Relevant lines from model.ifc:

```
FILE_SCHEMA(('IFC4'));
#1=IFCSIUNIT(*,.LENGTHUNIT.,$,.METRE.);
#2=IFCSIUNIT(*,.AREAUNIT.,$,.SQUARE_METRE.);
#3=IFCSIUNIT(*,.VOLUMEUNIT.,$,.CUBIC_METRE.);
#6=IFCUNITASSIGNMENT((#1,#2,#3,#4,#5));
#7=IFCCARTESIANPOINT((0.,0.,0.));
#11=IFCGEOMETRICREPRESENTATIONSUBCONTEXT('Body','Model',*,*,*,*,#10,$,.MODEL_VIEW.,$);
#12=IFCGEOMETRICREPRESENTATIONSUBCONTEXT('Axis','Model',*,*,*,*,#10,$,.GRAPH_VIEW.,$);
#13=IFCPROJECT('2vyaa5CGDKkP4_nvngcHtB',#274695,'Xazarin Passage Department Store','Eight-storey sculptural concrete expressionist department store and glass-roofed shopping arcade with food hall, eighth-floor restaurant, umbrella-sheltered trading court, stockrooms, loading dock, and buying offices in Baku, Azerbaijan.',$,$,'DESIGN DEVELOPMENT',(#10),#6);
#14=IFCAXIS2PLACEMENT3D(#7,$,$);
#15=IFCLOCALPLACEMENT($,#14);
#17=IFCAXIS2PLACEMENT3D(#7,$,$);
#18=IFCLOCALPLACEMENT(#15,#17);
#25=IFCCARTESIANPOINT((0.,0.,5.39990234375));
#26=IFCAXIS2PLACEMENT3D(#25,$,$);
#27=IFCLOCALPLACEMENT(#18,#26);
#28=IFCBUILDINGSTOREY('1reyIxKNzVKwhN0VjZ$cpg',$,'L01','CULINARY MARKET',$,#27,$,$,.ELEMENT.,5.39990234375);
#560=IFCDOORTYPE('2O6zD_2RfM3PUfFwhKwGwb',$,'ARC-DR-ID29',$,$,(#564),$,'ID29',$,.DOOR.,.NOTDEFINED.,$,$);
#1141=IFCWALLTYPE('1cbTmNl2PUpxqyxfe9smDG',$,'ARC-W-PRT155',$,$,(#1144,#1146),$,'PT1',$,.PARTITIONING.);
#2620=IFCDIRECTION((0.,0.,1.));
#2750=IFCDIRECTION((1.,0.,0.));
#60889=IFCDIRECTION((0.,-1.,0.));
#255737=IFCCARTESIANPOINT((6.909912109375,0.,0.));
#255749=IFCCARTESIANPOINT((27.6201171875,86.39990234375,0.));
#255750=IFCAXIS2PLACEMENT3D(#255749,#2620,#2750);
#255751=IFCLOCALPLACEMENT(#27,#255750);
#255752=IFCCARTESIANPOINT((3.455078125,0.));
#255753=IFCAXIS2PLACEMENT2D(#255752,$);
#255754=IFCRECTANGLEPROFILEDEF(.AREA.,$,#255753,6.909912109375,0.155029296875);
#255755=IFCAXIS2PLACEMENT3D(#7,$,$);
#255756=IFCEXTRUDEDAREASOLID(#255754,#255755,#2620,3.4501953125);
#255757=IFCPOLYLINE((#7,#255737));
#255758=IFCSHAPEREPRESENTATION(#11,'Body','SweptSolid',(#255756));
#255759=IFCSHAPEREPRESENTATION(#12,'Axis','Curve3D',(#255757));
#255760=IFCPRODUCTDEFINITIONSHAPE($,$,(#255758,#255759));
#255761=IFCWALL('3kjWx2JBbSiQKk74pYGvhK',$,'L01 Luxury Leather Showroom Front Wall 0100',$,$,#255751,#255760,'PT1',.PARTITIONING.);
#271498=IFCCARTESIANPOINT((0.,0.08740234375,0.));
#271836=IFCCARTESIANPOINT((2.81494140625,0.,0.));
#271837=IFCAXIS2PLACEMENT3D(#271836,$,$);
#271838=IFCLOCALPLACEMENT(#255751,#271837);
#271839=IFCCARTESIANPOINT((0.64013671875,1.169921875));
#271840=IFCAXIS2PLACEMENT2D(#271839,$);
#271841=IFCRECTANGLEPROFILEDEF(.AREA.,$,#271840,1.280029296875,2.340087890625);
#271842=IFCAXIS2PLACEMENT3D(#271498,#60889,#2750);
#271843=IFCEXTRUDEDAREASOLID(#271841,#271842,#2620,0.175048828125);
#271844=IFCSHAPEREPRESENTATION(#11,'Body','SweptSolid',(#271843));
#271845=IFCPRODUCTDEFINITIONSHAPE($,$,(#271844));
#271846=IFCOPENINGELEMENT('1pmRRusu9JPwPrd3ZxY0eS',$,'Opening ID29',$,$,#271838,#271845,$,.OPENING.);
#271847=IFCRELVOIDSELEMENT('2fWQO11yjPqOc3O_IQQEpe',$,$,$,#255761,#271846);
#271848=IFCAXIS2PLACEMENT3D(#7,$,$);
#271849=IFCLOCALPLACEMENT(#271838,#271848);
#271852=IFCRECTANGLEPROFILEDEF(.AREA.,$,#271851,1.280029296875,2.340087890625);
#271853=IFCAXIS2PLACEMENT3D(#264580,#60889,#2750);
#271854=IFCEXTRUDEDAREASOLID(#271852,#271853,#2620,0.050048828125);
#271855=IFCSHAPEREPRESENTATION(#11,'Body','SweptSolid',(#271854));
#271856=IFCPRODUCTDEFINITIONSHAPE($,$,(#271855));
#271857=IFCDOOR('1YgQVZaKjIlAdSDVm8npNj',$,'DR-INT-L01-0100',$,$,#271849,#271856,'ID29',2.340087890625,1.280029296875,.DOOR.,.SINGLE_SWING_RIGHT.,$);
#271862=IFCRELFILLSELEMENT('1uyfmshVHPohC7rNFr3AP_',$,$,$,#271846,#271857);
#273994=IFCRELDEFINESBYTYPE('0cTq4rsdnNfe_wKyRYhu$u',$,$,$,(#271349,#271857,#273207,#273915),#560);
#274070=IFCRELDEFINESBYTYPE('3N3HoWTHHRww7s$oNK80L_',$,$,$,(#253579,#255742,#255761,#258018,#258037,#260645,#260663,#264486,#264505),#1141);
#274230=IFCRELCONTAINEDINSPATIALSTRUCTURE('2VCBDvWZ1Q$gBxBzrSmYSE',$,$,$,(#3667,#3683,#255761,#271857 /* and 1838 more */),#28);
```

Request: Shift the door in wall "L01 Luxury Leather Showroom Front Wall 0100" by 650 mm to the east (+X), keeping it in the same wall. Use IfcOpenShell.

```python
import ifcopenshell
import ifcopenshell.api.geometry
import ifcopenshell.util.placement
import ifcopenshell.util.unit

model = ifcopenshell.open("model.ifc")
unit_scale = ifcopenshell.util.unit.calculate_unit_scale(model)

door = model.by_id(271857)
opening = door.FillsVoids[0].RelatingOpeningElement
wall = opening.VoidsElements[0].RelatingBuildingElement

wall_matrix = ifcopenshell.util.placement.get_local_placement(wall.ObjectPlacement)
shift = wall_matrix[:3, 0] * 0.65 / unit_scale
before = ifcopenshell.util.placement.get_local_placement(door.ObjectPlacement)[:3, 3].copy()

# The door is placed relative to its opening, so it follows when the opening moves.
matrix = ifcopenshell.util.placement.get_local_placement(opening.ObjectPlacement)
matrix[:3, 3] += shift
ifcopenshell.api.geometry.edit_object_placement(
    model, product=opening, matrix=matrix, is_si=False, should_transform_children=True
)

after = ifcopenshell.util.placement.get_local_placement(door.ObjectPlacement)[:3, 3]
print("door moved by", (after - before).round(3) + 0.0)

model.write("model_rev.ifc")
```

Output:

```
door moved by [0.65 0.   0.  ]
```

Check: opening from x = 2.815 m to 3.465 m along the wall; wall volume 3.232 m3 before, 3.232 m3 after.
